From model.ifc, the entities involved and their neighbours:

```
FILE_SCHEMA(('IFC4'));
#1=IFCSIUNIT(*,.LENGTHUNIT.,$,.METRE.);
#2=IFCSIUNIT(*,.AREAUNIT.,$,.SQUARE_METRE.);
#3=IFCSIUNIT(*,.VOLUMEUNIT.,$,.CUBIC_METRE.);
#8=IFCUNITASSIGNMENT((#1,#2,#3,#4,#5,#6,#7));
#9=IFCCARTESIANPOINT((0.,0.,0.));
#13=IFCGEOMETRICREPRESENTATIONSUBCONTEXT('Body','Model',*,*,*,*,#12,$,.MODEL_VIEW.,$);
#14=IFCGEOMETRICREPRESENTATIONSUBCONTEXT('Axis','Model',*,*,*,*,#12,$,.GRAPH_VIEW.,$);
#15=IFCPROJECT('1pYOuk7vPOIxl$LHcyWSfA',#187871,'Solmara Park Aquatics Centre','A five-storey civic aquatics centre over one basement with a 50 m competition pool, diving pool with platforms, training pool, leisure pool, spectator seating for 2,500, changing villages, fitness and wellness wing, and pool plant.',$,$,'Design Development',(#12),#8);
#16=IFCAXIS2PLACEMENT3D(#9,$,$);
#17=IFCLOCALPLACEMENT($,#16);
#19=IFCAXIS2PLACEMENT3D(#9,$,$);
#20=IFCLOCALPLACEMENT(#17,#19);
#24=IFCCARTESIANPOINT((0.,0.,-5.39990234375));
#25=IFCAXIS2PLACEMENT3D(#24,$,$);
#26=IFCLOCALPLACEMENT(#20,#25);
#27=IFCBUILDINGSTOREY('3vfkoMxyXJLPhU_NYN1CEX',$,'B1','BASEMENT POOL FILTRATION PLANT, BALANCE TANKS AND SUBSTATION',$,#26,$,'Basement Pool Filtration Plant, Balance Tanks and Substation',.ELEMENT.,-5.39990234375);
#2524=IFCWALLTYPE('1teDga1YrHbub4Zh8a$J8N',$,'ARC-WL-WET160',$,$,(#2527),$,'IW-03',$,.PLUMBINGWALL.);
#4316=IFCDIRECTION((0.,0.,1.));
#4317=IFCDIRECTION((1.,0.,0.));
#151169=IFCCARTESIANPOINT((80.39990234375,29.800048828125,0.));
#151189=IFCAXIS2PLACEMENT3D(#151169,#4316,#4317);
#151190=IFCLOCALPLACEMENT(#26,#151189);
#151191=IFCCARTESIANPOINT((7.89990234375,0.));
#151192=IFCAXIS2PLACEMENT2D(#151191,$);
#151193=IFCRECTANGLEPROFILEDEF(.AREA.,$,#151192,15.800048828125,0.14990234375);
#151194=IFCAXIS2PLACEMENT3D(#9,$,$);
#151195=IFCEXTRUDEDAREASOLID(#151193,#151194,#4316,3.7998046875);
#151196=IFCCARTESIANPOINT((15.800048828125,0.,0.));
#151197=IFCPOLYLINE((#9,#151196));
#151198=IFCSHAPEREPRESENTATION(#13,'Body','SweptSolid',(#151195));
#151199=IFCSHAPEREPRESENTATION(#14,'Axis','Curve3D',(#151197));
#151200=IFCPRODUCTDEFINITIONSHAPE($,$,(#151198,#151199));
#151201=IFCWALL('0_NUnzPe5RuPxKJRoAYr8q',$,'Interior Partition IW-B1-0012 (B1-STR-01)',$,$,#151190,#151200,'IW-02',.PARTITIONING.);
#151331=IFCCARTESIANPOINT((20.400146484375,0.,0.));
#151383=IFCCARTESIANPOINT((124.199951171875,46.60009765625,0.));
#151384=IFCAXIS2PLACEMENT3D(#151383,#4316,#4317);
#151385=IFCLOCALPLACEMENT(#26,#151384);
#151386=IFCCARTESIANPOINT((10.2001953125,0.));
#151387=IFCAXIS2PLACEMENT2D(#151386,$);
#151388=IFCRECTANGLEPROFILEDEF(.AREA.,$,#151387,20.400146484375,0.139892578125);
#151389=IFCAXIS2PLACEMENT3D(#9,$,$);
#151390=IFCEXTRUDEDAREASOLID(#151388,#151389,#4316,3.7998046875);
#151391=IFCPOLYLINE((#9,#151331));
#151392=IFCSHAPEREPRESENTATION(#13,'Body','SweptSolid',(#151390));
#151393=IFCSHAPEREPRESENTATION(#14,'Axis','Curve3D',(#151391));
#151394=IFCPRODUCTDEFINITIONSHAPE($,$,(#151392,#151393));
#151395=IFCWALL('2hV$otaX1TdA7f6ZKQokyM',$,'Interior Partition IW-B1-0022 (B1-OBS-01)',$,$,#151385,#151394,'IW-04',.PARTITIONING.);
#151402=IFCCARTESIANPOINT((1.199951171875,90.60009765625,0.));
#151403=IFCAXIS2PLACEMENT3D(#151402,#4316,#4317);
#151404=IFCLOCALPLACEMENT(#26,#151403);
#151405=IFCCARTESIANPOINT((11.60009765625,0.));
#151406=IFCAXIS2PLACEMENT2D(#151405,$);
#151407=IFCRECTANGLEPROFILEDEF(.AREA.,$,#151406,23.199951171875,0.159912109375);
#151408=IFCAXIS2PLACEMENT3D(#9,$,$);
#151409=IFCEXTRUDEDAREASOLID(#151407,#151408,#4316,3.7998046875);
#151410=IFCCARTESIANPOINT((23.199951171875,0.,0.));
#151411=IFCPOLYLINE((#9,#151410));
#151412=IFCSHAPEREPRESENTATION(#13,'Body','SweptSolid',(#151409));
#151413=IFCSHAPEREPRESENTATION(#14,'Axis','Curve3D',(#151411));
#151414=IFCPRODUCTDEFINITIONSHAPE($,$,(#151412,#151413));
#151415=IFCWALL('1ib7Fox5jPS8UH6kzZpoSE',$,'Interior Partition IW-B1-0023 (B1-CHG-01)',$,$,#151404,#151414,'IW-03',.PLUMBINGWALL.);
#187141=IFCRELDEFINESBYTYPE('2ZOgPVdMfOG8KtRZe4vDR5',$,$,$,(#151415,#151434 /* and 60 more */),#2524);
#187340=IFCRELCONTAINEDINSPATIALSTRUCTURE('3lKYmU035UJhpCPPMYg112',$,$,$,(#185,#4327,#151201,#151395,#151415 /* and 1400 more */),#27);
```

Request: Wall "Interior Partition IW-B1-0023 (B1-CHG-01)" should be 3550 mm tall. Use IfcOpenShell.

```python
import ifcopenshell
import ifcopenshell.geom
import ifcopenshell.util.representation
import ifcopenshell.util.shape
import ifcopenshell.util.unit

model = ifcopenshell.open("model.ifc")
unit_scale = ifcopenshell.util.unit.calculate_unit_scale(model)
settings = ifcopenshell.geom.settings()


def volume(element):
    """Net volume in cubic metres, openings subtracted."""
    shape = ifcopenshell.geom.create_shape(settings, element)
    return ifcopenshell.util.shape.get_volume(shape.geometry)


wall = model.by_guid("1ib7Fox5jPS8UH6kzZpoSE")
before = volume(wall)

body = ifcopenshell.util.representation.get_representation(wall, "Model", "Body")
solid = body.Items[0]
old_height = solid.Depth
solid.Depth = 3.55 / unit_scale
after = volume(wall)

print(f"height {old_height:g} -> {solid.Depth:g}, volume {before:.3f} -> {after:.3f} m3")

model.write("model_edited.ifc")
```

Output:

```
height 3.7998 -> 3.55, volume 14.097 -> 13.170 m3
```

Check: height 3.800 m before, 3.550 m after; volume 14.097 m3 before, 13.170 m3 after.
